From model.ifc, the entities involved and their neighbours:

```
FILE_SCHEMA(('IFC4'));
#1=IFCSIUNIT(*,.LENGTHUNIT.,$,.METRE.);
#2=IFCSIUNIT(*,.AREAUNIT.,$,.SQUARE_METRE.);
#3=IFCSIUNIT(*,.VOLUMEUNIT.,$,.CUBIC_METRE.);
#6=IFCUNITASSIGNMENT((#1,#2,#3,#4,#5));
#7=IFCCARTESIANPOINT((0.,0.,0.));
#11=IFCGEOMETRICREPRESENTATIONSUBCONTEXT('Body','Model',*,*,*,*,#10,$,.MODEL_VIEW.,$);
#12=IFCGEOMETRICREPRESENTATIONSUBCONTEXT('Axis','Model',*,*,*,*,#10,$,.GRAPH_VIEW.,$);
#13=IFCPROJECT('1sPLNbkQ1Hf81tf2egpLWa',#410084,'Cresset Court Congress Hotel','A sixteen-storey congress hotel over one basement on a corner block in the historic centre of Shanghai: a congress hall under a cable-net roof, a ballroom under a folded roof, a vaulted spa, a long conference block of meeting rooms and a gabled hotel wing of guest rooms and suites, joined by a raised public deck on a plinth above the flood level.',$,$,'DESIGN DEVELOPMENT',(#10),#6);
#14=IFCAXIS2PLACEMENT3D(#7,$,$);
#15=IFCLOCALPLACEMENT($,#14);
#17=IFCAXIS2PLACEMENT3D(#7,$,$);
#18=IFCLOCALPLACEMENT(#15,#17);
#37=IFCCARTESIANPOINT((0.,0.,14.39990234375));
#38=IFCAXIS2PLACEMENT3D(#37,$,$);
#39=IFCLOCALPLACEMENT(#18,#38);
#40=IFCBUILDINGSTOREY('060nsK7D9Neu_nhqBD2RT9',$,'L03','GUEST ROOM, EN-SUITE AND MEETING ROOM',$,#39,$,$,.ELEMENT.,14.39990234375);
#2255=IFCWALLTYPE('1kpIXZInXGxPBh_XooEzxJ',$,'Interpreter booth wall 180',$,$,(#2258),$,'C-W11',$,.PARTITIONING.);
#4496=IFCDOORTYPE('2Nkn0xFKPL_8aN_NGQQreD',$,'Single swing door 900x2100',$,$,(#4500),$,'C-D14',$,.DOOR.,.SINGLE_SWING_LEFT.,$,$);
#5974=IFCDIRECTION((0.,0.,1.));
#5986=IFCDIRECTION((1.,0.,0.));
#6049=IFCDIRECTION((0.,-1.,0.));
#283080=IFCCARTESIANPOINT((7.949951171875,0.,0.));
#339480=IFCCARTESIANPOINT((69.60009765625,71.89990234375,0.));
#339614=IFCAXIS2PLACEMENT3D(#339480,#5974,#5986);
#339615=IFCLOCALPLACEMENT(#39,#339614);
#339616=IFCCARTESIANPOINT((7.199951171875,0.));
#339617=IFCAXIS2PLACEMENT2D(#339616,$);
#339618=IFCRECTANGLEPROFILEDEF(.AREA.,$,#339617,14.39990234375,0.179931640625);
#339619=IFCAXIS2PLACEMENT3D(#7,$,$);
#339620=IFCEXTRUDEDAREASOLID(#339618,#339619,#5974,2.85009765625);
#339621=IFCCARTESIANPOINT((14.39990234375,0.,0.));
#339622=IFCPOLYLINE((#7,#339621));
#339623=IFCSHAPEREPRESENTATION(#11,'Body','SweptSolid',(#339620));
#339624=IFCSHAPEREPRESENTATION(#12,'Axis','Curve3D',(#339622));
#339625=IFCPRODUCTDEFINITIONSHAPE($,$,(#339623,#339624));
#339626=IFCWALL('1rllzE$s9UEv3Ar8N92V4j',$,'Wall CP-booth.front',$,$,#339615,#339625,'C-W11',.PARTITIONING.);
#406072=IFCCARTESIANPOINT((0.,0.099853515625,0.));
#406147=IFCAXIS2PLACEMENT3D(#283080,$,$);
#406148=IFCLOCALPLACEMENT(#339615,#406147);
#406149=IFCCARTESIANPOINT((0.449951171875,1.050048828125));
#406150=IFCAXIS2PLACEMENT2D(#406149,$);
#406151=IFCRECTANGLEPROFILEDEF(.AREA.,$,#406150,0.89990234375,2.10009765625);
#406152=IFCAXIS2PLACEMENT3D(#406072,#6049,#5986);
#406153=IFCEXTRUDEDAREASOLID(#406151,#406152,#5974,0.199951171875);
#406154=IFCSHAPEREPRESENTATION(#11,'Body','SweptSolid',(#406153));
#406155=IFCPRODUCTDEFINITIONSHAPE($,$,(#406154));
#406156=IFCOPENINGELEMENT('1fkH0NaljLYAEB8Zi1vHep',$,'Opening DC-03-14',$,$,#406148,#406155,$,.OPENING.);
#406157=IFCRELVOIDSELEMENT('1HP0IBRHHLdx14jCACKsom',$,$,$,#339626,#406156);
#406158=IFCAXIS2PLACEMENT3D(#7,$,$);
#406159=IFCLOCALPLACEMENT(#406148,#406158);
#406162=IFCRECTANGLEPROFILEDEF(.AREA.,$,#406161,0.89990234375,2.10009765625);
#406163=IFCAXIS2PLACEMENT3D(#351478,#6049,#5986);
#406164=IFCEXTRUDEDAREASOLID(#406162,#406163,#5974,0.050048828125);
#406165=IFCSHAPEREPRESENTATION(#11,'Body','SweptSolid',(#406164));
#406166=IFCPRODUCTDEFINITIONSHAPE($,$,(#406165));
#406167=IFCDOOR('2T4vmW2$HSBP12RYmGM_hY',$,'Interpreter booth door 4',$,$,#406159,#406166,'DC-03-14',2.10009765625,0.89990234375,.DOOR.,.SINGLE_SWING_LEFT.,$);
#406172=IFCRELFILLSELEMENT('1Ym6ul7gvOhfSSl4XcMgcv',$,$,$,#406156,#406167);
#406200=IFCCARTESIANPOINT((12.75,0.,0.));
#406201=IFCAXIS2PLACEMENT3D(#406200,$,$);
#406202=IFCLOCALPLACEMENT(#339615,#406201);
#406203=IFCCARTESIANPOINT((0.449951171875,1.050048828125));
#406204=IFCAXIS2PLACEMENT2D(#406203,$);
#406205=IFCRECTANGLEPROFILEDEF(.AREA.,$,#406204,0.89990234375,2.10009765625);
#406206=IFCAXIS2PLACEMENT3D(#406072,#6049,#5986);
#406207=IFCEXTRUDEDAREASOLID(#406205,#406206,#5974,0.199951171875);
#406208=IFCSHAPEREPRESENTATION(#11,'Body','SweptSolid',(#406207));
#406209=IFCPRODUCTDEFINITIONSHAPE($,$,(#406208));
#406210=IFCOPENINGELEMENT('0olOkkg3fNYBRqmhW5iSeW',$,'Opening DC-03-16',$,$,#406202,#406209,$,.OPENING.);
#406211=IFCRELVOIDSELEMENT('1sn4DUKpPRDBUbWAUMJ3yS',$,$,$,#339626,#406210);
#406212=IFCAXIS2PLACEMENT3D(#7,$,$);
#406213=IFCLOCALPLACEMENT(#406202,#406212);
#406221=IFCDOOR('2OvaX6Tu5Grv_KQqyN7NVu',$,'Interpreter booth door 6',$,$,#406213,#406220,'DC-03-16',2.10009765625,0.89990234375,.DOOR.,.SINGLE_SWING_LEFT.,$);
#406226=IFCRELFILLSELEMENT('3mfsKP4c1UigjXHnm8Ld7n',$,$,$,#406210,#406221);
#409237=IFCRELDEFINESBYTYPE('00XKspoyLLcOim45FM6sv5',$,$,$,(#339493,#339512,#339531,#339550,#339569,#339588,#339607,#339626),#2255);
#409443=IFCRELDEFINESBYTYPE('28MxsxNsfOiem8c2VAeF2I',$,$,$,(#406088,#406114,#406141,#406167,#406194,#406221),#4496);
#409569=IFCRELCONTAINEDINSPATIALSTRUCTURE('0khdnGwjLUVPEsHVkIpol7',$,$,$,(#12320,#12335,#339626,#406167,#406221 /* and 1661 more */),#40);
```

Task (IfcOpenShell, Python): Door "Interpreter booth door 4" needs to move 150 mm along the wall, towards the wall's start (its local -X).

```python
import ifcopenshell
import ifcopenshell.api.geometry
import ifcopenshell.util.placement

model = ifcopenshell.open("model.ifc")

door = model.by_guid("2T4vmW2$HSBP12RYmGM_hY")
opening = door.FillsVoids[0].RelatingOpeningElement
wall = opening.VoidsElements[0].RelatingBuildingElement

wall_matrix = ifcopenshell.util.placement.get_local_placement(wall.ObjectPlacement)
shift = wall_matrix[:3, 0] * -0.15
before = ifcopenshell.util.placement.get_local_placement(door.ObjectPlacement)[:3, 3].copy()

# The door is placed relative to its opening, so it follows when the opening moves.
matrix = ifcopenshell.util.placement.get_local_placement(opening.ObjectPlacement)
matrix[:3, 3] += shift
ifcopenshell.api.geometry.edit_object_placement(
    model, product=opening, matrix=matrix, is_si=False, should_transform_children=True
)

after = ifcopenshell.util.placement.get_local_placement(door.ObjectPlacement)[:3, 3]
print("door moved by", (after - before).round(3) + 0.0)

model.write("model-out.ifc")
```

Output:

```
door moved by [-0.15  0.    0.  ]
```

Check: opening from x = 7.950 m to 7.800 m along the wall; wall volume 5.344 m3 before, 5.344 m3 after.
